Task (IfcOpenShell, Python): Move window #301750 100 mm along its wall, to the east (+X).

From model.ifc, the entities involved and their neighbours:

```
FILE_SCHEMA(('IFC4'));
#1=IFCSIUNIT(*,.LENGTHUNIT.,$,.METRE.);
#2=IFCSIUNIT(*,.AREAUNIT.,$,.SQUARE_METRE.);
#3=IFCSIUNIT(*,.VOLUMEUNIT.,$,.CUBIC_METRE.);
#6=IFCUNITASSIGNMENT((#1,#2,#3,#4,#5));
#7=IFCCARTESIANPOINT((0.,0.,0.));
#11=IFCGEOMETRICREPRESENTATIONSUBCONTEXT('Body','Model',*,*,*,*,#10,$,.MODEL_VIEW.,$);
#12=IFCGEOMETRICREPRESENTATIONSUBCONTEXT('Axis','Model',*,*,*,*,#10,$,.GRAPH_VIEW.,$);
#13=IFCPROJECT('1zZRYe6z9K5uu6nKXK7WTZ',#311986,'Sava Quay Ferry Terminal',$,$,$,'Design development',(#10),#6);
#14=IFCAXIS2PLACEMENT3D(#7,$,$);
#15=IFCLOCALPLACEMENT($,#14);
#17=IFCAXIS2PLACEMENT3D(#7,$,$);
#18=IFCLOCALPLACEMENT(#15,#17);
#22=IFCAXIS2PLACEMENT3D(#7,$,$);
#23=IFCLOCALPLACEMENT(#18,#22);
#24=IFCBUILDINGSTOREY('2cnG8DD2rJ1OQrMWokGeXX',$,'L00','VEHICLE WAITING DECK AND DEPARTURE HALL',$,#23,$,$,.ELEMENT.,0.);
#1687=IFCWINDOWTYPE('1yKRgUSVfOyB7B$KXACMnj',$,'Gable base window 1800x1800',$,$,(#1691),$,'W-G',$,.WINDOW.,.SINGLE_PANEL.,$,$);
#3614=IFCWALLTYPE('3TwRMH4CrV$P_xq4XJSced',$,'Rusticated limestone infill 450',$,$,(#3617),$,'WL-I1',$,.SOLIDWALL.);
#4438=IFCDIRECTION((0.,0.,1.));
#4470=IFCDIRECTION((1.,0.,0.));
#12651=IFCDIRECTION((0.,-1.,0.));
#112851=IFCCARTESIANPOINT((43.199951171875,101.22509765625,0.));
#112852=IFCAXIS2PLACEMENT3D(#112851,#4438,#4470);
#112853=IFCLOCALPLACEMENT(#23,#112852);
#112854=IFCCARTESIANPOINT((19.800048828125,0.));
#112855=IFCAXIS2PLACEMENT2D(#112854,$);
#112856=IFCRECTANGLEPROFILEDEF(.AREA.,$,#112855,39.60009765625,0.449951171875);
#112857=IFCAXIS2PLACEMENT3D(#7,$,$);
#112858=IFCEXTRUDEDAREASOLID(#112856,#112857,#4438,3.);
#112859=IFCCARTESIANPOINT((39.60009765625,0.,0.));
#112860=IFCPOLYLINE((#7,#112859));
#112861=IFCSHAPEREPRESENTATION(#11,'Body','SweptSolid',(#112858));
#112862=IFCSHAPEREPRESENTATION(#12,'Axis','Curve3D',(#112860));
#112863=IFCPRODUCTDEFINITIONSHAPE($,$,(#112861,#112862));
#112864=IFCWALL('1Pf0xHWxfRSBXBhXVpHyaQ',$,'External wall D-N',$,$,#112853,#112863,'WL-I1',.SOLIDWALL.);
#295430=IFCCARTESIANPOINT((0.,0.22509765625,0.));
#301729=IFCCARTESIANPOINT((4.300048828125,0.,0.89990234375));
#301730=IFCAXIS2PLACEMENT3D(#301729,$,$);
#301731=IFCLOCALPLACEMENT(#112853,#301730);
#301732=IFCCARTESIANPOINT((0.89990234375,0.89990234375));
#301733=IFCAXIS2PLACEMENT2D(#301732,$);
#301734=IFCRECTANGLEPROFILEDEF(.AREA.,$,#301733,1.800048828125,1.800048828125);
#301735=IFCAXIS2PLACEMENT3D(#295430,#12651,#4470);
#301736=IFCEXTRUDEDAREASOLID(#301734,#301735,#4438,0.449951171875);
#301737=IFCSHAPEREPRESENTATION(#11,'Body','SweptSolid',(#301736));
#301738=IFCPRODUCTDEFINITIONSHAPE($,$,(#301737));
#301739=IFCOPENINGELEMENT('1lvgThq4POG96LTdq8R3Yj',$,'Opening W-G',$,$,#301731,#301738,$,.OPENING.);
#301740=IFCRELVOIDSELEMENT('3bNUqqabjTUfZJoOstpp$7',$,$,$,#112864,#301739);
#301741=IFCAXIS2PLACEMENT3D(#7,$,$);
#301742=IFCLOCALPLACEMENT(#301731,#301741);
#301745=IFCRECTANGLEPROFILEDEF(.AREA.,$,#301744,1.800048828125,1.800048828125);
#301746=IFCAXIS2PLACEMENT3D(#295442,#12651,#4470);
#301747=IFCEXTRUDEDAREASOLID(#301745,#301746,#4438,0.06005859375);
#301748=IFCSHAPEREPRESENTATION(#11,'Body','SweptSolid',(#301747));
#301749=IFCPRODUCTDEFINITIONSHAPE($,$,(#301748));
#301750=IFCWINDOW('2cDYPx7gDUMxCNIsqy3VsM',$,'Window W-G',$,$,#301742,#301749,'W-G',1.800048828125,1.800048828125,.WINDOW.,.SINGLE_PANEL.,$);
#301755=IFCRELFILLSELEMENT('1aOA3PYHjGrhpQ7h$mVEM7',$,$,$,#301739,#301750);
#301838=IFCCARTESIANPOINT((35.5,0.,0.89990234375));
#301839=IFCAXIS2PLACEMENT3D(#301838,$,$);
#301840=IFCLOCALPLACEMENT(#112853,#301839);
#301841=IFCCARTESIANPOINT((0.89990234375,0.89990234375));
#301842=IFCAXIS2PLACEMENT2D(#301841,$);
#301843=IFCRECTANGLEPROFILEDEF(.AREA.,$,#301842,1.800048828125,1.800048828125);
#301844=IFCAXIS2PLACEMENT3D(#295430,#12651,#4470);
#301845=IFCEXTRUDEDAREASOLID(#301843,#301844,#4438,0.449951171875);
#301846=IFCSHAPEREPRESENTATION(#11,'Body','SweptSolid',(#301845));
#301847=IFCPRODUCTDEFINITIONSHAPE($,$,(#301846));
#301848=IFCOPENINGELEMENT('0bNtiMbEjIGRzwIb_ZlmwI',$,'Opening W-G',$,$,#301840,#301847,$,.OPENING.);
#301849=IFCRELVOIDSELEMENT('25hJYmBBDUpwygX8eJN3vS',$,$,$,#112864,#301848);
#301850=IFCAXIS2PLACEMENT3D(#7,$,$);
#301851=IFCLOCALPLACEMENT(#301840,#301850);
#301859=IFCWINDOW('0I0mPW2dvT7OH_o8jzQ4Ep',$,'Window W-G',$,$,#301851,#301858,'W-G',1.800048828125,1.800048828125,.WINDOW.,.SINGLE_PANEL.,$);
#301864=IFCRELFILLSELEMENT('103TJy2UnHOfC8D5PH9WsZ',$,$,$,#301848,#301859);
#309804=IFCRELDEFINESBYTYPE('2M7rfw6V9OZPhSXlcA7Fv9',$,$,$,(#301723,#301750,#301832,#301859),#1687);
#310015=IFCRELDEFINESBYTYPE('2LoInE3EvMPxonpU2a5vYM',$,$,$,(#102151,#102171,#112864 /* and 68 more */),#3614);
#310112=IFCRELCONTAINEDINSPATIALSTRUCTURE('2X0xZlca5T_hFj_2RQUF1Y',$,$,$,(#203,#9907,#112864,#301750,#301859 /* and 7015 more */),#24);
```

```python
import ifcopenshell
import ifcopenshell.api.geometry
import ifcopenshell.util.placement
import ifcopenshell.util.unit

model = ifcopenshell.open("model.ifc")
unit_scale = ifcopenshell.util.unit.calculate_unit_scale(model)

window = model.by_guid("2cDYPx7gDUMxCNIsqy3VsM")
opening = window.FillsVoids[0].RelatingOpeningElement
wall = opening.VoidsElements[0].RelatingBuildingElement

wall_matrix = ifcopenshell.util.placement.get_local_placement(wall.ObjectPlacement)
shift = wall_matrix[:3, 0] * 0.1 / unit_scale
before = ifcopenshell.util.placement.get_local_placement(window.ObjectPlacement)[:3, 3].copy()

# The window is placed relative to its opening, so it follows when the opening moves.
matrix = ifcopenshell.util.placement.get_local_placement(opening.ObjectPlacement)
matrix[:3, 3] += shift
ifcopenshell.api.geometry.edit_object_placement(
    model, product=opening, matrix=matrix, is_si=False, should_transform_children=True
)

after = ifcopenshell.util.placement.get_local_placement(window.ObjectPlacement)[:3, 3]
print("window moved by", (after - before).round(3) + 0.0)

model.write("model_v2.ifc")
```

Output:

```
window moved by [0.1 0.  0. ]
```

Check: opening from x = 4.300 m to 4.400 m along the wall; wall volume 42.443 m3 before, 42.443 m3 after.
